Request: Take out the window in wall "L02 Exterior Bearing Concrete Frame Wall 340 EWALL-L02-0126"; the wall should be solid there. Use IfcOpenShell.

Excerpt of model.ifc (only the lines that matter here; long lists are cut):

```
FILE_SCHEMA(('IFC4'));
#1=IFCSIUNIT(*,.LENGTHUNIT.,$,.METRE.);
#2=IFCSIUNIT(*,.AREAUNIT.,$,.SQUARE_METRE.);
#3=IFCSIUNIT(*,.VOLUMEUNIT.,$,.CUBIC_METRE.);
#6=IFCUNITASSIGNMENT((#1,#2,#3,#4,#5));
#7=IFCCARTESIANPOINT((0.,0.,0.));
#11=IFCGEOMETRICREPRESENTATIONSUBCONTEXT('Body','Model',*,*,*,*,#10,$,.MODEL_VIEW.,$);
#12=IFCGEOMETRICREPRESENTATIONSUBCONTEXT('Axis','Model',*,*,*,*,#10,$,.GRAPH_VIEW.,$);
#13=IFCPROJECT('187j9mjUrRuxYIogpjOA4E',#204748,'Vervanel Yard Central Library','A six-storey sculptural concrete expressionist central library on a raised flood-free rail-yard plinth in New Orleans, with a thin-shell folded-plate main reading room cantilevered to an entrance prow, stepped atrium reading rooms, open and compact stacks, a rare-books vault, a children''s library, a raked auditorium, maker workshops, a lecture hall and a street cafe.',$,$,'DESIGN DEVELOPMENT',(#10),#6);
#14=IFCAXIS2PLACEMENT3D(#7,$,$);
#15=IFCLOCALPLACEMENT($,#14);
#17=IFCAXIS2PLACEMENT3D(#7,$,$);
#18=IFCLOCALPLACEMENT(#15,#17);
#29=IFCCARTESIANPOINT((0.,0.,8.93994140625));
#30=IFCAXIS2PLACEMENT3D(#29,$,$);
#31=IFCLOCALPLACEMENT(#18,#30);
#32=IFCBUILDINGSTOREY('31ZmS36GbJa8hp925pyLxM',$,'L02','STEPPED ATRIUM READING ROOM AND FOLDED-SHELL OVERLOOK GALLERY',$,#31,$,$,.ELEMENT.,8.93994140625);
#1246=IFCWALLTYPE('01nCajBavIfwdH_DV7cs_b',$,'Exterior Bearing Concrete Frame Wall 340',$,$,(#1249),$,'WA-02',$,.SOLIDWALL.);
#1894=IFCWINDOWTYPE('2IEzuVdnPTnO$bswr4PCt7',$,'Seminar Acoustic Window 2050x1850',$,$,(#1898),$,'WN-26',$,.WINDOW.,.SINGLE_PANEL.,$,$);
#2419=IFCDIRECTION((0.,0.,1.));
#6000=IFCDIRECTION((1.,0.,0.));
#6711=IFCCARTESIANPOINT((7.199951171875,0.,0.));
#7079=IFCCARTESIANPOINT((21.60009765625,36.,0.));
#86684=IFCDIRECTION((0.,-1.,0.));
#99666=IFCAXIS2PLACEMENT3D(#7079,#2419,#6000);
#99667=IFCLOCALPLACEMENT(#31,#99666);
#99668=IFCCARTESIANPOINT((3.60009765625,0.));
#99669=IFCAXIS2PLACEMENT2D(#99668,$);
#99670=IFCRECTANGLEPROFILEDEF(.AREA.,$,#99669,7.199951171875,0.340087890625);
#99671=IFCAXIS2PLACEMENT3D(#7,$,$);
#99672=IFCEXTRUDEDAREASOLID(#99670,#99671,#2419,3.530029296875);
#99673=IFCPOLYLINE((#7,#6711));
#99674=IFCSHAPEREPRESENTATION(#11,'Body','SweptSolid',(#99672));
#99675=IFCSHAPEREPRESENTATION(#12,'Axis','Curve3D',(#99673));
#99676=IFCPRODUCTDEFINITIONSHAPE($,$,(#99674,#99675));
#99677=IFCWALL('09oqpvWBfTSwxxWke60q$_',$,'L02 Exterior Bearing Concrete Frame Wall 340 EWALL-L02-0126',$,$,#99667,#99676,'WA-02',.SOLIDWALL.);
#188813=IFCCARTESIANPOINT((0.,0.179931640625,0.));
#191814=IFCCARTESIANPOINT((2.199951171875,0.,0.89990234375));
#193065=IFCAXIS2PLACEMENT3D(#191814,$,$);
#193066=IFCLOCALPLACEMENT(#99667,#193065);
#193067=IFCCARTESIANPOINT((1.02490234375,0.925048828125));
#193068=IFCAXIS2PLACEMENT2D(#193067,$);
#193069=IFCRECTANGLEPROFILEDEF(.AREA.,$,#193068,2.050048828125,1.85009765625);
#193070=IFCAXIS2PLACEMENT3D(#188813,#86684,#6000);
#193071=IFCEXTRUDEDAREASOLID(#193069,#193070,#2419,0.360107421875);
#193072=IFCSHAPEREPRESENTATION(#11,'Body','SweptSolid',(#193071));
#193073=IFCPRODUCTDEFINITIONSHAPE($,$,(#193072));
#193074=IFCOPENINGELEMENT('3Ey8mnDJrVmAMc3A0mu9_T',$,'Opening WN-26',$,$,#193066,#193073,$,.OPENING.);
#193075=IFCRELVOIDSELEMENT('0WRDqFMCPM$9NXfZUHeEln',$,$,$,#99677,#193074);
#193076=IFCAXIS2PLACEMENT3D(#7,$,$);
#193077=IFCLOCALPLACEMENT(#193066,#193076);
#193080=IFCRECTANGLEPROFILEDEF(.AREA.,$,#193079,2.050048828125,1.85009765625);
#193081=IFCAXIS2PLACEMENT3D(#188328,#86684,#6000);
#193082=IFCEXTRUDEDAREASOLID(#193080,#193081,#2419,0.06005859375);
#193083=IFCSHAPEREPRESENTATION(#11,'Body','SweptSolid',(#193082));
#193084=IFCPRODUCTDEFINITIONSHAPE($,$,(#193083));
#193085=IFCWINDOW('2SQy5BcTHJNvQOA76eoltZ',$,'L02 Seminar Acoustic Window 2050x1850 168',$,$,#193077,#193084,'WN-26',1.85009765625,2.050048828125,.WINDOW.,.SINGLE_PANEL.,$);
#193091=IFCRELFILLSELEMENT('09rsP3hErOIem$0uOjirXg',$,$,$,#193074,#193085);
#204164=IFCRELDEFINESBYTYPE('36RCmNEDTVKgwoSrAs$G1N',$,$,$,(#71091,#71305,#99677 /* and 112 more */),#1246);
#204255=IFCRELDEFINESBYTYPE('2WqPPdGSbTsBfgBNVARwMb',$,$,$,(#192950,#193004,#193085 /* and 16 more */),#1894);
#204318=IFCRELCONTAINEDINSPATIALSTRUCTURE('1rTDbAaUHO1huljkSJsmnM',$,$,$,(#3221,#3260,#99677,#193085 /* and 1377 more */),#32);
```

```python
import ifcopenshell
import ifcopenshell.api.feature
import ifcopenshell.api.root
import ifcopenshell.geom
import ifcopenshell.util.shape

model = ifcopenshell.open("model.ifc")
settings = ifcopenshell.geom.settings()


def volume(element):
    """Net volume in cubic metres, openings subtracted."""
    shape = ifcopenshell.geom.create_shape(settings, element)
    return ifcopenshell.util.shape.get_volume(shape.geometry)


window = model.by_guid("2SQy5BcTHJNvQOA76eoltZ")
opening = window.FillsVoids[0].RelatingOpeningElement
wall = opening.VoidsElements[0].RelatingBuildingElement
before = volume(wall)

ifcopenshell.api.root.remove_product(model, product=window)
ifcopenshell.api.feature.remove_feature(model, feature=opening)

after = volume(wall)

print(f"wall volume {before:.3f} -> {after:.3f} m3")

model.write("model_v2.ifc")
```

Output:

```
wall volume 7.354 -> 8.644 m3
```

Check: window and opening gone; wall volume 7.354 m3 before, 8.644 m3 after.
